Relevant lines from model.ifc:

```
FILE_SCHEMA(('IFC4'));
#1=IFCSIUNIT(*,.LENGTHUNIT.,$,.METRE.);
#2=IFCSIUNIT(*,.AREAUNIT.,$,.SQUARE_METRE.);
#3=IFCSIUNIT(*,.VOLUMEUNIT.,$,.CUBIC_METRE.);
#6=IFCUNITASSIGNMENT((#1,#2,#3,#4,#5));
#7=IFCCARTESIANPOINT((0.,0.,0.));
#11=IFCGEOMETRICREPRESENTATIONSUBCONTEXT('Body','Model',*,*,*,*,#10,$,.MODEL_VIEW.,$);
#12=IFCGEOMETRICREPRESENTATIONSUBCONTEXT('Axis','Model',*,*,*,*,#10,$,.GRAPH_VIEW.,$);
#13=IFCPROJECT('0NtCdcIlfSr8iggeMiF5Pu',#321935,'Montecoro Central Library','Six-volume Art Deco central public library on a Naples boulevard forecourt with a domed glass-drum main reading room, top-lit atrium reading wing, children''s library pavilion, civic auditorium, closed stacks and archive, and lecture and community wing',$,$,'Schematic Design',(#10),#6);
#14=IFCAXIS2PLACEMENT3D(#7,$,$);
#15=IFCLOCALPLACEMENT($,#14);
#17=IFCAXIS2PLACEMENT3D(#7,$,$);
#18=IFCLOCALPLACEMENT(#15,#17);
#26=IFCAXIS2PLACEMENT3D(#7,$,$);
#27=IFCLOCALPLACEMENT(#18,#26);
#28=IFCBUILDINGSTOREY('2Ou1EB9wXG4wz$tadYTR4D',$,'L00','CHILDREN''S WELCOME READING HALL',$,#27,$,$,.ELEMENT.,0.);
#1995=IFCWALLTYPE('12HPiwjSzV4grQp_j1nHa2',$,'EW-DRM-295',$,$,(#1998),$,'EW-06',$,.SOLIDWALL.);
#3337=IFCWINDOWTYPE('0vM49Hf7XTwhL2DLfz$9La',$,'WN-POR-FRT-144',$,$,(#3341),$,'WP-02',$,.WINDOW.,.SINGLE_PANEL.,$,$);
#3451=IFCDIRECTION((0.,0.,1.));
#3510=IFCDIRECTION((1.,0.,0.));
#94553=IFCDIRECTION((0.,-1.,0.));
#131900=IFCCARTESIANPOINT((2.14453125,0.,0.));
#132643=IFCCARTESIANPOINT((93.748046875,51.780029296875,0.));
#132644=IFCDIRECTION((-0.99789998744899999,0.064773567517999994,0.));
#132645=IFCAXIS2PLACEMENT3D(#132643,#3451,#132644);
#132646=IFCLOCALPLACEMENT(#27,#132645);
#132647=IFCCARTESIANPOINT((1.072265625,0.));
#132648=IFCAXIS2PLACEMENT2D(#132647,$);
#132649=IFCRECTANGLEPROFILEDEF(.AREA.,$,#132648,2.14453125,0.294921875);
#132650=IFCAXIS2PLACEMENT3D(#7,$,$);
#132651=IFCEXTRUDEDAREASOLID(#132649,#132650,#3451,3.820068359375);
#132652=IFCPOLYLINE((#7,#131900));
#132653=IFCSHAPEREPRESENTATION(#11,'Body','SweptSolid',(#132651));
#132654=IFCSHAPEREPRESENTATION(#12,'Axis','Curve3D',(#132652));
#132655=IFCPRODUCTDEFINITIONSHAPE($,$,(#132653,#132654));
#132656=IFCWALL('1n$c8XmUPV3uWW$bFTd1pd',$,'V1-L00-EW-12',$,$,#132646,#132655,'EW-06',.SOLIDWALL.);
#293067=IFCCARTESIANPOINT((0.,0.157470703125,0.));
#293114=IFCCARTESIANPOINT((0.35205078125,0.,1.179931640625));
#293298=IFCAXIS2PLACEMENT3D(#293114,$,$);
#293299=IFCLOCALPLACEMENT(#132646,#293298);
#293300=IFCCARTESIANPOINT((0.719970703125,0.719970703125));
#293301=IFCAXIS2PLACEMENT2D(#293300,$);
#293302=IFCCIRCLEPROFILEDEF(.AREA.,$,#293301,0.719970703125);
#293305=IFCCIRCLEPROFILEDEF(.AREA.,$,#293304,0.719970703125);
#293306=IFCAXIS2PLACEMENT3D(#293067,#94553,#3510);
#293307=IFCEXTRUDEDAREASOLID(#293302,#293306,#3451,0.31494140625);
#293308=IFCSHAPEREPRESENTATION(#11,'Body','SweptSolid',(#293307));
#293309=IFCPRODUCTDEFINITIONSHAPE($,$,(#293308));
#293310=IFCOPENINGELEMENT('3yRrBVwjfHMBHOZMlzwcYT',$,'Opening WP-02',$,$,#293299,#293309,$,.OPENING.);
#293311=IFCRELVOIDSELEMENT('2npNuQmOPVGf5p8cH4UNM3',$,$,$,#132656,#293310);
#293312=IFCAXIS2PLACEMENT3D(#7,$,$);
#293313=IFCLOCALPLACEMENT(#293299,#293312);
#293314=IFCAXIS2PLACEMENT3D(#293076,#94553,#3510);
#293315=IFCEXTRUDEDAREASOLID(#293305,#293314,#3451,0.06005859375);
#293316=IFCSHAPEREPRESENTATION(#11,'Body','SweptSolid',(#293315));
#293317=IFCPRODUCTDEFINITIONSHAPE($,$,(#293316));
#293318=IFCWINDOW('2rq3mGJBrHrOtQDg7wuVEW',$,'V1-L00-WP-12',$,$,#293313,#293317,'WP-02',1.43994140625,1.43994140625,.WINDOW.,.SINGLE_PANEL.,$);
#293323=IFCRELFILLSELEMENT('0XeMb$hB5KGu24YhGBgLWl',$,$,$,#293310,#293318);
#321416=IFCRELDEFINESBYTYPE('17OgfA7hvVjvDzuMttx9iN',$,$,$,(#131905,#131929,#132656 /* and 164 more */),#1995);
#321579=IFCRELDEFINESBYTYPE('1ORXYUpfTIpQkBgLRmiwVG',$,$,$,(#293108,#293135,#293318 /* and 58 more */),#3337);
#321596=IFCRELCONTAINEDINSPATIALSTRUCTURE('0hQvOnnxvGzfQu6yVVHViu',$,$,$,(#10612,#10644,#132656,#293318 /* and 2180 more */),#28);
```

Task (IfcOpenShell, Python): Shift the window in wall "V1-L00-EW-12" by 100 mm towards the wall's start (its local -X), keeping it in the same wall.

```python
import ifcopenshell
import ifcopenshell.api.geometry
import ifcopenshell.util.placement
import ifcopenshell.util.unit

model = ifcopenshell.open("model.ifc")
unit_scale = ifcopenshell.util.unit.calculate_unit_scale(model)

window = model.by_guid("2rq3mGJBrHrOtQDg7wuVEW")
opening = window.FillsVoids[0].RelatingOpeningElement
wall = opening.VoidsElements[0].RelatingBuildingElement

wall_matrix = ifcopenshell.util.placement.get_local_placement(wall.ObjectPlacement)
shift = wall_matrix[:3, 0] * -0.1 / unit_scale
before = ifcopenshell.util.placement.get_local_placement(window.ObjectPlacement)[:3, 3].copy()

# The window is placed relative to its opening, so it follows when the opening moves.
matrix = ifcopenshell.util.placement.get_local_placement(opening.ObjectPlacement)
matrix[:3, 3] += shift
ifcopenshell.api.geometry.edit_object_placement(
    model, product=opening, matrix=matrix, is_si=False, should_transform_children=True
)

after = ifcopenshell.util.placement.get_local_placement(window.ObjectPlacement)[:3, 3]
print("window moved by", (after - before).round(3) + 0.0)

model.write("model_rev.ifc")
```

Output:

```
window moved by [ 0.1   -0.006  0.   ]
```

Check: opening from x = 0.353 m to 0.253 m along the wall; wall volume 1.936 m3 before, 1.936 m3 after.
